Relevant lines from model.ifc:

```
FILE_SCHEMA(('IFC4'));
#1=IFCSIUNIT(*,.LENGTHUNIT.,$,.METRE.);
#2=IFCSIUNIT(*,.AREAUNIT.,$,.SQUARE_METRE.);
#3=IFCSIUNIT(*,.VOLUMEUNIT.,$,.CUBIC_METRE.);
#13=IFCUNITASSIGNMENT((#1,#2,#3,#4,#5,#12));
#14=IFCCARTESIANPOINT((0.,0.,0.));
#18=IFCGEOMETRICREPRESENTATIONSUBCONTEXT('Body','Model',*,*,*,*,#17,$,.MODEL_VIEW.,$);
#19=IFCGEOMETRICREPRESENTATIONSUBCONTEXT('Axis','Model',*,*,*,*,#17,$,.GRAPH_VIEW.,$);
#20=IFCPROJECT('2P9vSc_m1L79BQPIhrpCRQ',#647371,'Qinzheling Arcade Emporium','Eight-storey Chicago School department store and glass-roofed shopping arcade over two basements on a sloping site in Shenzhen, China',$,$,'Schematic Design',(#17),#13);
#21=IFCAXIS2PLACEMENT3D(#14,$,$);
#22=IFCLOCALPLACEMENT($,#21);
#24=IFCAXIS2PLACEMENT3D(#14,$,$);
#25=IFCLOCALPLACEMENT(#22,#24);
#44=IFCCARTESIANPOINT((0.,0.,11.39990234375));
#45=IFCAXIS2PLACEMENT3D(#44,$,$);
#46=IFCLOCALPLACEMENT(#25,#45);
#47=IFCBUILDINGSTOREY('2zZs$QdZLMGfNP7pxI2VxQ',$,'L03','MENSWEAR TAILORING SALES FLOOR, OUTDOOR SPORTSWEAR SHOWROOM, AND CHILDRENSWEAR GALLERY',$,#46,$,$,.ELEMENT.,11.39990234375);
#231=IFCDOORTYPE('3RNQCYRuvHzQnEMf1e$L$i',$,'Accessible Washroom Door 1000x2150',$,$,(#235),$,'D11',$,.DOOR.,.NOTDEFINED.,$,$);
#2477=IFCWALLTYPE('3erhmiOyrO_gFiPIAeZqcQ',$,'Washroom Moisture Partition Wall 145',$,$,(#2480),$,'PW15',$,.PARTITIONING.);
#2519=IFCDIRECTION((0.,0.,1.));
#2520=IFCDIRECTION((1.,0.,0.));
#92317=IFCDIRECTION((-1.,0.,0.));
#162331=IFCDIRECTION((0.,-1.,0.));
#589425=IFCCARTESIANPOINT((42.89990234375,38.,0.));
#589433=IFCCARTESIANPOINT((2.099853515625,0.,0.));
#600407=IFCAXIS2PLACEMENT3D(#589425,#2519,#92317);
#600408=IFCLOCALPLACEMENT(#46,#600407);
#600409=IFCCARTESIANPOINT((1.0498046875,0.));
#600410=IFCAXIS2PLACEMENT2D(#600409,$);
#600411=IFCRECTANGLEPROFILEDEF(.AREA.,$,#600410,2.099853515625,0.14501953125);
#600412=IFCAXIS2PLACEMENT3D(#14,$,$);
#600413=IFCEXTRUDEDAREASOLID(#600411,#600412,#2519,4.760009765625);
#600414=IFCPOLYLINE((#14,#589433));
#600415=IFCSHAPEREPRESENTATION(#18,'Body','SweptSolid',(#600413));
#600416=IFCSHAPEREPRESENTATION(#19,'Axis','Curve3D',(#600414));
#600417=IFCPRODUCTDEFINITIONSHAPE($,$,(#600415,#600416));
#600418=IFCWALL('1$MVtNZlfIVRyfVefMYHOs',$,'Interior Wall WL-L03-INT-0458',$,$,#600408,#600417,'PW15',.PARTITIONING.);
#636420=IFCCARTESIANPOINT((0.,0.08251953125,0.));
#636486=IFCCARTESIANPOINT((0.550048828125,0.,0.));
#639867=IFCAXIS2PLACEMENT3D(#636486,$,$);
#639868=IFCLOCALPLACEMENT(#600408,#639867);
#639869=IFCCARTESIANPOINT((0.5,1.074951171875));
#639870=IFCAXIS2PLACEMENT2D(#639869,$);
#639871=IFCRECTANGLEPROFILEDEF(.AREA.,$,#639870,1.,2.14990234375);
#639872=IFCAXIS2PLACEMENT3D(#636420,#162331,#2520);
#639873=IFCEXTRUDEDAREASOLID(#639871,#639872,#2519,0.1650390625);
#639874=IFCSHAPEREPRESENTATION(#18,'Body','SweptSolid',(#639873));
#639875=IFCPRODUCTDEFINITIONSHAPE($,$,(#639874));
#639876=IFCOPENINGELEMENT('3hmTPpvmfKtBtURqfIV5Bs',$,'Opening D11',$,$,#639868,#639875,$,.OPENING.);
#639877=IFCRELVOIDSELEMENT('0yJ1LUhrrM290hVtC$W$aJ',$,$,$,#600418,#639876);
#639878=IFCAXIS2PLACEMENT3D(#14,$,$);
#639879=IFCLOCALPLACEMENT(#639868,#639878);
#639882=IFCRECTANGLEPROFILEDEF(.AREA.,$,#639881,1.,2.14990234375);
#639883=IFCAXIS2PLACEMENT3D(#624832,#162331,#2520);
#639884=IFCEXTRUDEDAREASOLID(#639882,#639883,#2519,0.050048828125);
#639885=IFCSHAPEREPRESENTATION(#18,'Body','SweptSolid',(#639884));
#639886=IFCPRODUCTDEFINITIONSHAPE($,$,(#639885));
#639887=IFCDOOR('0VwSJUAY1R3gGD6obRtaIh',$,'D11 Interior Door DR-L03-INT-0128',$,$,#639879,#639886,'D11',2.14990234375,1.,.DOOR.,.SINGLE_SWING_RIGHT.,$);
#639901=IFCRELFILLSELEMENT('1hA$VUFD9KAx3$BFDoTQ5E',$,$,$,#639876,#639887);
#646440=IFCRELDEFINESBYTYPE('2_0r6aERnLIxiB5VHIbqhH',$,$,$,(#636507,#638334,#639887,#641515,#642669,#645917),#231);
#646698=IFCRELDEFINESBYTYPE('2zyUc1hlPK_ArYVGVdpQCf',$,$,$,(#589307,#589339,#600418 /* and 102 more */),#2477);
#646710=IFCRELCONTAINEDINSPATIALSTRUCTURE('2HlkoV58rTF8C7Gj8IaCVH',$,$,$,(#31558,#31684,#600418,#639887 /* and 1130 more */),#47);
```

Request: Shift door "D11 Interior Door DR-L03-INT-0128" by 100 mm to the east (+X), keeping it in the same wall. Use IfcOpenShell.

```python
import ifcopenshell
import ifcopenshell.api.geometry
import ifcopenshell.util.placement
import ifcopenshell.util.unit

model = ifcopenshell.open("model.ifc")
unit_scale = ifcopenshell.util.unit.calculate_unit_scale(model)

door = model.by_guid("0VwSJUAY1R3gGD6obRtaIh")
opening = door.FillsVoids[0].RelatingOpeningElement
wall = opening.VoidsElements[0].RelatingBuildingElement

wall_matrix = ifcopenshell.util.placement.get_local_placement(wall.ObjectPlacement)
shift = wall_matrix[:3, 0] * -0.1 / unit_scale
before = ifcopenshell.util.placement.get_local_placement(door.ObjectPlacement)[:3, 3].copy()

# The door is placed relative to its opening, so it follows when the opening moves.
matrix = ifcopenshell.util.placement.get_local_placement(opening.ObjectPlacement)
matrix[:3, 3] += shift
ifcopenshell.api.geometry.edit_object_placement(
    model, product=opening, matrix=matrix, is_si=False, should_transform_children=True
)

after = ifcopenshell.util.placement.get_local_placement(door.ObjectPlacement)[:3, 3]
print("door moved by", (after - before).round(3) + 0.0)

model.write("model-out.ifc")
```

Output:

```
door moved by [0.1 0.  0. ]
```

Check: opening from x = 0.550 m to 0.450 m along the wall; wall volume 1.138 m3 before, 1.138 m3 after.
